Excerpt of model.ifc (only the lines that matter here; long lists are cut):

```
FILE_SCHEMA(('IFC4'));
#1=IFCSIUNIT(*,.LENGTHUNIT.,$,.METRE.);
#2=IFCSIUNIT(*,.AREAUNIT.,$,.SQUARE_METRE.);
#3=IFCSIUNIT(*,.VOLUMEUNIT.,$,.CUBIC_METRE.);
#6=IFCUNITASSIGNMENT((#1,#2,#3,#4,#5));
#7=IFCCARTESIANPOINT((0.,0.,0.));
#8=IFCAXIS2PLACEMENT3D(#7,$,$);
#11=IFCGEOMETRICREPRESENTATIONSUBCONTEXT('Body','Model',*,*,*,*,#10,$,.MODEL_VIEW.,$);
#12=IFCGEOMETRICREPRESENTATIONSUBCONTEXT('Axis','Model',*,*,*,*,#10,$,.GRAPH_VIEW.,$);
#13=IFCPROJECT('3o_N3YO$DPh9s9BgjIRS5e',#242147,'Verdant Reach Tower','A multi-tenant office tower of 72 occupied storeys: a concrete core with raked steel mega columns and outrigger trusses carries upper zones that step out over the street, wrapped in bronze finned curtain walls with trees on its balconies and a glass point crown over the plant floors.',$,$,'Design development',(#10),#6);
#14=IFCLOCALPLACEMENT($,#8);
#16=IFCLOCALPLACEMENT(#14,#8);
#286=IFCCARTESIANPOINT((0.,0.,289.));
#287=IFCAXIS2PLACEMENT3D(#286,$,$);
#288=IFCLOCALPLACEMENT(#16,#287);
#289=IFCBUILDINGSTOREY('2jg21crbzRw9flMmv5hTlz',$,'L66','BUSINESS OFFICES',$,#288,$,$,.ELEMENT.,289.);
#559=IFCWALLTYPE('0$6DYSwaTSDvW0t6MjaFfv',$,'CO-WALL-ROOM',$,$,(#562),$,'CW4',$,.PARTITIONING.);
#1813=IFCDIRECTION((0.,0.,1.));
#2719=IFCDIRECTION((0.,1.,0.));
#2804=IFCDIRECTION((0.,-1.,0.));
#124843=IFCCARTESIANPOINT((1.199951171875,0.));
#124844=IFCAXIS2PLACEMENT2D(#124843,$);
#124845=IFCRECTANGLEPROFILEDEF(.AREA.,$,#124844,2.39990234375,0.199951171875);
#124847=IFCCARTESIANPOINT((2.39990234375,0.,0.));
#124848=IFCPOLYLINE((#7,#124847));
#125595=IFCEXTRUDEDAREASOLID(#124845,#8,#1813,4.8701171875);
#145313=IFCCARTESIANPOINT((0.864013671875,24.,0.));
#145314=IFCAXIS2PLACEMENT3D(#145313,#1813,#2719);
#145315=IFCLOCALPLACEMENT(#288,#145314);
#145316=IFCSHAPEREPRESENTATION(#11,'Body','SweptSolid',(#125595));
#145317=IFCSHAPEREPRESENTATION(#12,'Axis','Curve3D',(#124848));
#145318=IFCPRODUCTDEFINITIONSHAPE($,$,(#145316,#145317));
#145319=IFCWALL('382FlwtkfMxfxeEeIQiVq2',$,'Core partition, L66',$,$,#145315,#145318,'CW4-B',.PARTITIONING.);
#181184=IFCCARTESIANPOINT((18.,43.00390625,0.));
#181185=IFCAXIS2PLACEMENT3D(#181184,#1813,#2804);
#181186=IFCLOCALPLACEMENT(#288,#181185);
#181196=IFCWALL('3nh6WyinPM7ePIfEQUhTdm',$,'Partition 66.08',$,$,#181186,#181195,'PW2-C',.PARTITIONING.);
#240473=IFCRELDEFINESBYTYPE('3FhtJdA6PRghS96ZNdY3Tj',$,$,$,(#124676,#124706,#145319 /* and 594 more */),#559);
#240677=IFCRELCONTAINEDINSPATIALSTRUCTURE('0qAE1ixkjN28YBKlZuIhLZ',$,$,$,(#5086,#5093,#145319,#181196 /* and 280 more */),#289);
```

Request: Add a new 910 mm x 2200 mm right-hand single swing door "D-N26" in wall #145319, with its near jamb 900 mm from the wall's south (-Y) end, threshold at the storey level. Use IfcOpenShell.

```python
import numpy as np
import ifcopenshell
import ifcopenshell.api.feature
import ifcopenshell.api.geometry
import ifcopenshell.api.root
import ifcopenshell.api.spatial
import ifcopenshell.geom
import ifcopenshell.util.element
import ifcopenshell.util.placement
import ifcopenshell.util.representation
import ifcopenshell.util.shape
import ifcopenshell.util.unit

model = ifcopenshell.open("model.ifc")
unit_scale = ifcopenshell.util.unit.calculate_unit_scale(model)
settings = ifcopenshell.geom.settings()


def volume(element):
    """Net volume in cubic metres, openings subtracted."""
    shape = ifcopenshell.geom.create_shape(settings, element)
    return ifcopenshell.util.shape.get_volume(shape.geometry)


wall = model.by_guid("382FlwtkfMxfxeEeIQiVq2")
storey = ifcopenshell.util.element.get_container(wall, ifc_class="IfcBuildingStorey")
context = ifcopenshell.util.representation.get_context(model, "Model", "Body", "MODEL_VIEW")
before = volume(wall)

width, height, from_end, sill = 0.91, 2.2, 0.9, 0.0  # metres

# The wall runs along its own X axis, and the end named is its -X end.
wall_shape = ifcopenshell.geom.create_shape(settings, wall)
x, y, z = ifcopenshell.util.shape.get_vertices(wall_shape.geometry).T
start = x.min() + from_end
face, thickness = float(y.min()), float(y.max() - y.min())
wall_matrix = ifcopenshell.util.placement.get_local_placement(wall.ObjectPlacement)
level = ifcopenshell.util.placement.get_local_placement(storey.ObjectPlacement)[2, 3]


def in_wall(x, y):
    """Placement at x, y metres in the wall's axes, at sill height."""
    matrix = wall_matrix.copy()
    matrix[:, 3] = wall_matrix @ np.array([x / unit_scale, y / unit_scale, 0.0, 1.0])
    matrix[2, 3] = level + sill / unit_scale
    return matrix


# Opening: a box that overshoots both wall faces by 50 mm.
opening = ifcopenshell.api.root.create_entity(model, ifc_class="IfcOpeningElement", predefined_type="OPENING")
box = ifcopenshell.api.geometry.add_wall_representation(
    model, context=context, length=width, height=height, thickness=thickness + 0.1
)
ifcopenshell.api.geometry.assign_representation(model, product=opening, representation=box)
ifcopenshell.api.geometry.edit_object_placement(model, product=opening, matrix=in_wall(start, face - 0.05), is_si=False)
ifcopenshell.api.feature.add_feature(model, feature=opening, element=wall)

door = ifcopenshell.api.root.create_entity(model, ifc_class="IfcDoor", name="D-N26", predefined_type="DOOR")
door.OverallWidth, door.OverallHeight = width / unit_scale, height / unit_scale
door.OperationType = "SINGLE_SWING_RIGHT"
body = ifcopenshell.api.geometry.add_door_representation(
    model,
    context=context,
    overall_width=door.OverallWidth,
    overall_height=door.OverallHeight,
    operation_type="SINGLE_SWING_RIGHT",
    lining_properties={"LiningDepth": thickness / unit_scale, "ThresholdDepth": thickness / unit_scale},
)
ifcopenshell.api.geometry.assign_representation(model, product=door, representation=body)
ifcopenshell.api.spatial.assign_container(model, products=[door], relating_structure=storey)
ifcopenshell.api.feature.add_filling(model, opening=opening, element=door)

# The lining spans the wall, so the door starts at the wall face.
ifcopenshell.api.geometry.edit_object_placement(model, product=door, matrix=in_wall(start, face), is_si=False)

after = volume(wall)

print(f"wall volume {before:.3f} -> {after:.3f} m3")

model.write("model_updated.ifc")
```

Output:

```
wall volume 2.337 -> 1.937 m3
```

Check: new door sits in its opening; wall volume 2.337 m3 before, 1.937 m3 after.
